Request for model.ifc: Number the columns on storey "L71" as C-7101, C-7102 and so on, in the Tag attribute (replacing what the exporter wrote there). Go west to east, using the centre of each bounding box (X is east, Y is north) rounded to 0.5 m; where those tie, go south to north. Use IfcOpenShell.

First a look at what the model holds.

```python
import ifcopenshell
import ifcopenshell.util.element
import ifcopenshell.util.placement

model = ifcopenshell.open("model.ifc")
print(model.schema)
storey = next(s for s in model.by_type("IfcBuildingStorey") if s.Name == "L71")
columns = [e for e in ifcopenshell.util.element.get_decomposition(storey) if e.is_a("IfcColumn")]
for e in sorted(columns, key=lambda e: e.id()):
    origin = ifcopenshell.util.placement.get_local_placement(e.ObjectPlacement)[:3, 3]
    print(e.id(), e.Tag, e.Name, origin.round(2) + 0.0, sep=" | ")
```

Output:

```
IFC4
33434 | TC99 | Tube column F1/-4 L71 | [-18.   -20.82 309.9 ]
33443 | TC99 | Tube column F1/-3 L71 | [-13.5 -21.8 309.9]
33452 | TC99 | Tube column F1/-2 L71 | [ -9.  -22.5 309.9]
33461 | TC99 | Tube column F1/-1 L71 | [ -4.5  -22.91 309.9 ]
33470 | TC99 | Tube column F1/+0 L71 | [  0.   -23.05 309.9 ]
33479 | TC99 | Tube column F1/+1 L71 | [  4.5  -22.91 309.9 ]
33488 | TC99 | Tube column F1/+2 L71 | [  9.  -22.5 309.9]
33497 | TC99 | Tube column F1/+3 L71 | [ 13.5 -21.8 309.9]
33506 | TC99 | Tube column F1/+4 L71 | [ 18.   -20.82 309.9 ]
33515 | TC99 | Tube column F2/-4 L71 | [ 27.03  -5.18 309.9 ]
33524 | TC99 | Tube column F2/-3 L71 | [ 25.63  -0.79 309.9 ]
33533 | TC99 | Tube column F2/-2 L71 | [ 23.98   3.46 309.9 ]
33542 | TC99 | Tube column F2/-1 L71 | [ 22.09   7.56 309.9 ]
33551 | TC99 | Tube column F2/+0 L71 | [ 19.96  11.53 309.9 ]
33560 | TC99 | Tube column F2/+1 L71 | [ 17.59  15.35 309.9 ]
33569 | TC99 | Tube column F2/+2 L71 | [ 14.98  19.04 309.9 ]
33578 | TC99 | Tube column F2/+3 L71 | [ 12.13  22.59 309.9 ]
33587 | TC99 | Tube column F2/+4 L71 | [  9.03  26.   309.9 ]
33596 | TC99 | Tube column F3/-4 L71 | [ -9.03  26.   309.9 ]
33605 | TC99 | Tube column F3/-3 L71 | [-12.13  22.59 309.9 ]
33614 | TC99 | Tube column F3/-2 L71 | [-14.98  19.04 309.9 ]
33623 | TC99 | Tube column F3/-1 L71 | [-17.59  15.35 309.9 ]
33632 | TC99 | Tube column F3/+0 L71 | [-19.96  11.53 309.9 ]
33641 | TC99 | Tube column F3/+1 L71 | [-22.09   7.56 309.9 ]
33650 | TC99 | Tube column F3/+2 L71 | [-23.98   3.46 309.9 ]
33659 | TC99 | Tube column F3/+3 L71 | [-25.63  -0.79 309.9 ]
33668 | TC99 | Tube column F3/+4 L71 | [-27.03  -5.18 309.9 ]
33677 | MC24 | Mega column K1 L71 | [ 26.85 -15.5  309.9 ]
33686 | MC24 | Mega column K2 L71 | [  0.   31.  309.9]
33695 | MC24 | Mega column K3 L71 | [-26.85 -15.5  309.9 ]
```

```python
import ifcopenshell
import ifcopenshell.geom
import ifcopenshell.util.element
import ifcopenshell.util.shape

model = ifcopenshell.open("model.ifc")
settings = ifcopenshell.geom.settings()
settings.set("use-world-coords", True)


def centre(element):
    shape = ifcopenshell.geom.create_shape(settings, element)
    return ifcopenshell.util.shape.get_bbox_centroid(shape.geometry)


storey = next(s for s in model.by_type("IfcBuildingStorey") if s.Name == "L71")
columns = [e for e in ifcopenshell.util.element.get_decomposition(storey) if e.is_a("IfcColumn")]

# Insertion points can sit at a corner or the storey origin, so sort by the geometry (in metres).
centres = {e: centre(e) for e in columns}
columns.sort(key=lambda e: (round(centres[e][0] / 0.5), centres[e][1]))

for i, e in enumerate(columns, start=1):
    number = f"C-71{i:02d}"
    e.Tag = number
    print(e.id(), number)

model.write("model-out.ifc")
```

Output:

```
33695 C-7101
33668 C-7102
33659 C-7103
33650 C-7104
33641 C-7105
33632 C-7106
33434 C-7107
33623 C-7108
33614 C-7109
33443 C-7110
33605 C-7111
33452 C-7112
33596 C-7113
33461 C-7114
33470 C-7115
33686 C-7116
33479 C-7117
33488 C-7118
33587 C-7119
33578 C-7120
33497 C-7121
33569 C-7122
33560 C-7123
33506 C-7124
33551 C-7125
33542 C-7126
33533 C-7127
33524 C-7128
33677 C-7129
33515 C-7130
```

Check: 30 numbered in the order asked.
